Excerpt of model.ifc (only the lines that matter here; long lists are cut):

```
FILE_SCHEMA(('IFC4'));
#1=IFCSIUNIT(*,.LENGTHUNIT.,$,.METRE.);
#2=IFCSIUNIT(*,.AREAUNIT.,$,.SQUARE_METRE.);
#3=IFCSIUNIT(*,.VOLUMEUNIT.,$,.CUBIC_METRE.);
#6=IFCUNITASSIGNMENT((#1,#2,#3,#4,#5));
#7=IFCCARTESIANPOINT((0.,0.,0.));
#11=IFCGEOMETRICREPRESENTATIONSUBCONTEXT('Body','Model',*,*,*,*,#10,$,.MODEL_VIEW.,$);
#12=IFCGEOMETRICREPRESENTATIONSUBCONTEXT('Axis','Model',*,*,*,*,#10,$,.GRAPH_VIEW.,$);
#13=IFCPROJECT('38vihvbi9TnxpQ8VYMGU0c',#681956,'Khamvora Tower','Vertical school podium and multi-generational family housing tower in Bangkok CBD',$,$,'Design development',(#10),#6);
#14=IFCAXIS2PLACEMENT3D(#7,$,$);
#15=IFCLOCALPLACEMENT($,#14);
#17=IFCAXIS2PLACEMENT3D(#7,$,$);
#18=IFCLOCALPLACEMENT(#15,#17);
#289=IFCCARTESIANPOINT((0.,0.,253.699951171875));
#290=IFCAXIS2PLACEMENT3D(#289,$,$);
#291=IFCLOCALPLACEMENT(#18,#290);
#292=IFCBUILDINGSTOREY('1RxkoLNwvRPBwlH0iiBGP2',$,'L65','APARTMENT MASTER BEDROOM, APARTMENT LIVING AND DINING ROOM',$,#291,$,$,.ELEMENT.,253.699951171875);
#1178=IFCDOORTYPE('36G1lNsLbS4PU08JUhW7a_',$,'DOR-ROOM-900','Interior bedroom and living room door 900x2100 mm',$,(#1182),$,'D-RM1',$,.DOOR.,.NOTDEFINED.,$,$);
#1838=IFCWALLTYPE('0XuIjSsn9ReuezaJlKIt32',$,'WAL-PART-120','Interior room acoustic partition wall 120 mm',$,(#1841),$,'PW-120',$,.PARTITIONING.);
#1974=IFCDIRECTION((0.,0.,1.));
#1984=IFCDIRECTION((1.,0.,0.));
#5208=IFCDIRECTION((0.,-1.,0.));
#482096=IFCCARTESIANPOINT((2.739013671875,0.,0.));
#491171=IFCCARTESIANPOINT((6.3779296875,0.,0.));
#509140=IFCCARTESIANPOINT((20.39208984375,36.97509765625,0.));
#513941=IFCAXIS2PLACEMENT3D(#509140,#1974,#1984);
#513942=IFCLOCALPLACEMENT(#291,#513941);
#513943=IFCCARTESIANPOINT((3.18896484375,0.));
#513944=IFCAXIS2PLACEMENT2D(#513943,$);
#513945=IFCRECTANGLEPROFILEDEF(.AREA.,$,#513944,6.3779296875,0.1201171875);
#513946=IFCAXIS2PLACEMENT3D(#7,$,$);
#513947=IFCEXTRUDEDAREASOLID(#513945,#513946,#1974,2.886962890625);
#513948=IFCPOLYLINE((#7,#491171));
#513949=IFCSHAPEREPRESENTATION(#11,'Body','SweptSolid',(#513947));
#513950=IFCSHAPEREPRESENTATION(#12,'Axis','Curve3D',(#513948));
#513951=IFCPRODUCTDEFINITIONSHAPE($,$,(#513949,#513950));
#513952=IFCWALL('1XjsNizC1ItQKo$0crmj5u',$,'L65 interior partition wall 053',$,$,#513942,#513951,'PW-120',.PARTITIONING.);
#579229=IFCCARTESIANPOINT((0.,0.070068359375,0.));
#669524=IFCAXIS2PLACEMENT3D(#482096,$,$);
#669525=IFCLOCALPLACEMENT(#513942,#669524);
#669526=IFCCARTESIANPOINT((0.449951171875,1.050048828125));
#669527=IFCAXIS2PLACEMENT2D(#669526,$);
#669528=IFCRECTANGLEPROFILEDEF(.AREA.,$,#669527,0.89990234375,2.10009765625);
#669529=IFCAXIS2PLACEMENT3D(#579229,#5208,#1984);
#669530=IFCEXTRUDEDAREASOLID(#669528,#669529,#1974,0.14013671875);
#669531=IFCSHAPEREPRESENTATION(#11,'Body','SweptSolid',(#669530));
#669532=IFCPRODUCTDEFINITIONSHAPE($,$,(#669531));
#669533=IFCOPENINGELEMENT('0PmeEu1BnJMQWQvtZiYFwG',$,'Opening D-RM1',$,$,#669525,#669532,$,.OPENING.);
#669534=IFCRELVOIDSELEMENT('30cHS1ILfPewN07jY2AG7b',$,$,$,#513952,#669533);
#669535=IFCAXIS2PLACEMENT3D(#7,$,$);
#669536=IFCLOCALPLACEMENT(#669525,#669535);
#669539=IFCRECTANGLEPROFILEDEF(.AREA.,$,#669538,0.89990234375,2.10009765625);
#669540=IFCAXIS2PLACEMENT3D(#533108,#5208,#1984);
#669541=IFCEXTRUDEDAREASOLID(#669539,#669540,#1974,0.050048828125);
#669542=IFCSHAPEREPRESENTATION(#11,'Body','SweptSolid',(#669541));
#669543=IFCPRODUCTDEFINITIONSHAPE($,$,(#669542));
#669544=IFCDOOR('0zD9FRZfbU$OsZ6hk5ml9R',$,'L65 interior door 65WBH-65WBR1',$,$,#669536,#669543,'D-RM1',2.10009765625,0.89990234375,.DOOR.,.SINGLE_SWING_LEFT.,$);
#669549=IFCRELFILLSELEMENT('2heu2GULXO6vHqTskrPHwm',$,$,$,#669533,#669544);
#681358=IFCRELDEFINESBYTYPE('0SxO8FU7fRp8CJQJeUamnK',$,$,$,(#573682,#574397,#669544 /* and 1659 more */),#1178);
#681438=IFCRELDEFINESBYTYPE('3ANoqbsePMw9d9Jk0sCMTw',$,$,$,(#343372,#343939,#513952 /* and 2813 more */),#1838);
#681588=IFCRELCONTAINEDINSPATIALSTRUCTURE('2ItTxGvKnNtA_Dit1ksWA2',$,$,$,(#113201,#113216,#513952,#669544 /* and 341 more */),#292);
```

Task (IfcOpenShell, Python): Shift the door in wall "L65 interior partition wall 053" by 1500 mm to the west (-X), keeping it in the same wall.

```python
import ifcopenshell
import ifcopenshell.api.geometry
import ifcopenshell.util.placement
import ifcopenshell.util.unit

model = ifcopenshell.open("model.ifc")
unit_scale = ifcopenshell.util.unit.calculate_unit_scale(model)

door = model.by_guid("0zD9FRZfbU$OsZ6hk5ml9R")
opening = door.FillsVoids[0].RelatingOpeningElement
wall = opening.VoidsElements[0].RelatingBuildingElement

wall_matrix = ifcopenshell.util.placement.get_local_placement(wall.ObjectPlacement)
shift = wall_matrix[:3, 0] * -1.5 / unit_scale
before = ifcopenshell.util.placement.get_local_placement(door.ObjectPlacement)[:3, 3].copy()

# The door is placed relative to its opening, so it follows when the opening moves.
matrix = ifcopenshell.util.placement.get_local_placement(opening.ObjectPlacement)
matrix[:3, 3] += shift
ifcopenshell.api.geometry.edit_object_placement(
    model, product=opening, matrix=matrix, is_si=False, should_transform_children=True
)

after = ifcopenshell.util.placement.get_local_placement(door.ObjectPlacement)[:3, 3]
print("door moved by", (after - before).round(3) + 0.0)

model.write("model_edited.ifc")
```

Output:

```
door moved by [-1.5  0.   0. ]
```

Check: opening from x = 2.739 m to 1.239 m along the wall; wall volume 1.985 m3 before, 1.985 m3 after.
